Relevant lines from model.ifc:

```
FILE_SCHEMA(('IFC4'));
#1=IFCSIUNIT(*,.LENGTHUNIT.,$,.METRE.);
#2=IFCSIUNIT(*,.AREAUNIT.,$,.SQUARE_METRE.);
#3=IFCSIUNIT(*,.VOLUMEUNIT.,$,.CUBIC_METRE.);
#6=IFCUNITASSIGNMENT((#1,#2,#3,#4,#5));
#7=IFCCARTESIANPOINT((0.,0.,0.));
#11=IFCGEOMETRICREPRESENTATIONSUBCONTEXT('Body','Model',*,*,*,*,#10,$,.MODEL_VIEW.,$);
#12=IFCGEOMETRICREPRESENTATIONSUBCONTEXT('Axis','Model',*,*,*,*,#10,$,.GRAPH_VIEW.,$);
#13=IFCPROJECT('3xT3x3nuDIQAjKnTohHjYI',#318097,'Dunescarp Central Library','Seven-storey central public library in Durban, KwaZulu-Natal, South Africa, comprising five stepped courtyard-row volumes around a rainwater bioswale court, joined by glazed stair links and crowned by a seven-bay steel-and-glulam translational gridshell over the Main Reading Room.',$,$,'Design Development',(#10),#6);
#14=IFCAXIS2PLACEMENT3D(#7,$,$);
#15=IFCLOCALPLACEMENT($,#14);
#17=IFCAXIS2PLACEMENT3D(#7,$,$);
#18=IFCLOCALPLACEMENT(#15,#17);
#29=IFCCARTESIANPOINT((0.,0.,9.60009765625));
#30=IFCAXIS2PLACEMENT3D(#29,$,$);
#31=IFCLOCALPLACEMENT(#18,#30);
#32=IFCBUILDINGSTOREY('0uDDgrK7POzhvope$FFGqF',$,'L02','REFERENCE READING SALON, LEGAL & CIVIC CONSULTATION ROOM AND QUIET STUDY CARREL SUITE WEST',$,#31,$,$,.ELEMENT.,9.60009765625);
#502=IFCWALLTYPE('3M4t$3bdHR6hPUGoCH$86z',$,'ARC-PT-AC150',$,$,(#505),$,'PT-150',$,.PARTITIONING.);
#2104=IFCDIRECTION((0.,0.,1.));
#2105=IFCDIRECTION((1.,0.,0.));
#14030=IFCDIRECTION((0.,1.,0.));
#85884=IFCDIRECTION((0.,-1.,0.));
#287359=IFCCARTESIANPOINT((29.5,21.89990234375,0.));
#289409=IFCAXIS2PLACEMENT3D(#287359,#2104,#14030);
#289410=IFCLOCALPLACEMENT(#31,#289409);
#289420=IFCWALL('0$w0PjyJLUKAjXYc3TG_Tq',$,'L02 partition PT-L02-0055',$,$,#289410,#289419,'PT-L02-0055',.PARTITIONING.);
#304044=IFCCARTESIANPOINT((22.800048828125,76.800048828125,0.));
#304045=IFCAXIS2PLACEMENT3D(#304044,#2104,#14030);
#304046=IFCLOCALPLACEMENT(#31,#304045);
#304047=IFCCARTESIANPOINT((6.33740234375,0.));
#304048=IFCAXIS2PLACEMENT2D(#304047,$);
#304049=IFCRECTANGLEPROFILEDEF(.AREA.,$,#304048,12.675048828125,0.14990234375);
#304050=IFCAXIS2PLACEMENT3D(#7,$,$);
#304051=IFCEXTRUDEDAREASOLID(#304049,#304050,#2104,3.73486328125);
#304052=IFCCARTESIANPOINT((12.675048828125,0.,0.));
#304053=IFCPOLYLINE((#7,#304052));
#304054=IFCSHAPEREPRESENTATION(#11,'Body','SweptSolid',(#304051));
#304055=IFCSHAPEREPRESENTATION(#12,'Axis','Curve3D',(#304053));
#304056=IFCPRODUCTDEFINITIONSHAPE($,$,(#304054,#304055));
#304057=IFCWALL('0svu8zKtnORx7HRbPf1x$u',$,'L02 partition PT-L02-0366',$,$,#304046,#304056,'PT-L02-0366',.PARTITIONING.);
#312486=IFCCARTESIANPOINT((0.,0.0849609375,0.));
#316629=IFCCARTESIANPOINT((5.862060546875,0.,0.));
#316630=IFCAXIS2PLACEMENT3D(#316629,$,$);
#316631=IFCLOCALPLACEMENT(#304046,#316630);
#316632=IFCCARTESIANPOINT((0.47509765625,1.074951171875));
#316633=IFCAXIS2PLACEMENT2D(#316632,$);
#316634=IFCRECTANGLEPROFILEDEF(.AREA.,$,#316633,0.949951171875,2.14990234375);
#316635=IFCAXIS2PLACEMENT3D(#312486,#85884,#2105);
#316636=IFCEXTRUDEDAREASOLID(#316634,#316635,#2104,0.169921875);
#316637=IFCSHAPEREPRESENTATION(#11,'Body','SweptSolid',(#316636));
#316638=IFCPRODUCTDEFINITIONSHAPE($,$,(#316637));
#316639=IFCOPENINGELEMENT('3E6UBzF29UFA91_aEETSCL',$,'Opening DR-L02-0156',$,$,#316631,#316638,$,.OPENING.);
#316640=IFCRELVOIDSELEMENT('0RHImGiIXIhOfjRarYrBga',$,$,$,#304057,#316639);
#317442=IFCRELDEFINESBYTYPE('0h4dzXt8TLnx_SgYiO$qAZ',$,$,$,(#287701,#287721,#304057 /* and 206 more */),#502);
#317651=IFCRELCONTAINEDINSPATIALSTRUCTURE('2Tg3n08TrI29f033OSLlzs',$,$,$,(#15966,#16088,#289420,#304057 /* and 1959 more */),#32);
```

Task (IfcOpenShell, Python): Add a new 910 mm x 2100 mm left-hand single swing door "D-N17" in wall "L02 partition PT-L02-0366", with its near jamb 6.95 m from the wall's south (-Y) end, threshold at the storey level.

```python
import numpy as np
import ifcopenshell
import ifcopenshell.api.feature
import ifcopenshell.api.geometry
import ifcopenshell.api.root
import ifcopenshell.api.spatial
import ifcopenshell.geom
import ifcopenshell.util.element
import ifcopenshell.util.placement
import ifcopenshell.util.representation
import ifcopenshell.util.shape
import ifcopenshell.util.unit

model = ifcopenshell.open("model.ifc")
unit_scale = ifcopenshell.util.unit.calculate_unit_scale(model)
settings = ifcopenshell.geom.settings()


def volume(element):
    """Net volume in cubic metres, openings subtracted."""
    shape = ifcopenshell.geom.create_shape(settings, element)
    return ifcopenshell.util.shape.get_volume(shape.geometry)


wall = model.by_guid("0svu8zKtnORx7HRbPf1x$u")
storey = ifcopenshell.util.element.get_container(wall, ifc_class="IfcBuildingStorey")
context = ifcopenshell.util.representation.get_context(model, "Model", "Body", "MODEL_VIEW")
before = volume(wall)

width, height, from_end, sill = 0.91, 2.1, 6.95, 0.0  # metres

# The wall runs along its own X axis, and the end named is its -X end.
wall_shape = ifcopenshell.geom.create_shape(settings, wall)
x, y, z = ifcopenshell.util.shape.get_vertices(wall_shape.geometry).T
start = x.min() + from_end
face, thickness = float(y.min()), float(y.max() - y.min())
wall_matrix = ifcopenshell.util.placement.get_local_placement(wall.ObjectPlacement)
level = ifcopenshell.util.placement.get_local_placement(storey.ObjectPlacement)[2, 3]


def in_wall(x, y):
    """Placement at x, y metres in the wall's axes, at sill height."""
    matrix = wall_matrix.copy()
    matrix[:, 3] = wall_matrix @ np.array([x / unit_scale, y / unit_scale, 0.0, 1.0])
    matrix[2, 3] = level + sill / unit_scale
    return matrix


# Opening: a box that overshoots both wall faces by 50 mm.
opening = ifcopenshell.api.root.create_entity(model, ifc_class="IfcOpeningElement", predefined_type="OPENING")
box = ifcopenshell.api.geometry.add_wall_representation(
    model, context=context, length=width, height=height, thickness=thickness + 0.1
)
ifcopenshell.api.geometry.assign_representation(model, product=opening, representation=box)
ifcopenshell.api.geometry.edit_object_placement(model, product=opening, matrix=in_wall(start, face - 0.05), is_si=False)
ifcopenshell.api.feature.add_feature(model, feature=opening, element=wall)

door = ifcopenshell.api.root.create_entity(model, ifc_class="IfcDoor", name="D-N17", predefined_type="DOOR")
door.OverallWidth, door.OverallHeight = width / unit_scale, height / unit_scale
door.OperationType = "SINGLE_SWING_LEFT"
body = ifcopenshell.api.geometry.add_door_representation(
    model,
    context=context,
    overall_width=door.OverallWidth,
    overall_height=door.OverallHeight,
    operation_type="SINGLE_SWING_LEFT",
    lining_properties={"LiningDepth": thickness / unit_scale, "ThresholdDepth": thickness / unit_scale},
)
ifcopenshell.api.geometry.assign_representation(model, product=door, representation=body)
ifcopenshell.api.spatial.assign_container(model, products=[door], relating_structure=storey)
ifcopenshell.api.feature.add_filling(model, opening=opening, element=door)

# The lining spans the wall, so the door starts at the wall face.
ifcopenshell.api.geometry.edit_object_placement(model, product=door, matrix=in_wall(start, face), is_si=False)

after = volume(wall)

print(f"wall volume {before:.3f} -> {after:.3f} m3")

model.write("model_updated.ifc")
```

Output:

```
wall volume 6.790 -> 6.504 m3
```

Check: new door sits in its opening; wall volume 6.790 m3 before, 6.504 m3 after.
